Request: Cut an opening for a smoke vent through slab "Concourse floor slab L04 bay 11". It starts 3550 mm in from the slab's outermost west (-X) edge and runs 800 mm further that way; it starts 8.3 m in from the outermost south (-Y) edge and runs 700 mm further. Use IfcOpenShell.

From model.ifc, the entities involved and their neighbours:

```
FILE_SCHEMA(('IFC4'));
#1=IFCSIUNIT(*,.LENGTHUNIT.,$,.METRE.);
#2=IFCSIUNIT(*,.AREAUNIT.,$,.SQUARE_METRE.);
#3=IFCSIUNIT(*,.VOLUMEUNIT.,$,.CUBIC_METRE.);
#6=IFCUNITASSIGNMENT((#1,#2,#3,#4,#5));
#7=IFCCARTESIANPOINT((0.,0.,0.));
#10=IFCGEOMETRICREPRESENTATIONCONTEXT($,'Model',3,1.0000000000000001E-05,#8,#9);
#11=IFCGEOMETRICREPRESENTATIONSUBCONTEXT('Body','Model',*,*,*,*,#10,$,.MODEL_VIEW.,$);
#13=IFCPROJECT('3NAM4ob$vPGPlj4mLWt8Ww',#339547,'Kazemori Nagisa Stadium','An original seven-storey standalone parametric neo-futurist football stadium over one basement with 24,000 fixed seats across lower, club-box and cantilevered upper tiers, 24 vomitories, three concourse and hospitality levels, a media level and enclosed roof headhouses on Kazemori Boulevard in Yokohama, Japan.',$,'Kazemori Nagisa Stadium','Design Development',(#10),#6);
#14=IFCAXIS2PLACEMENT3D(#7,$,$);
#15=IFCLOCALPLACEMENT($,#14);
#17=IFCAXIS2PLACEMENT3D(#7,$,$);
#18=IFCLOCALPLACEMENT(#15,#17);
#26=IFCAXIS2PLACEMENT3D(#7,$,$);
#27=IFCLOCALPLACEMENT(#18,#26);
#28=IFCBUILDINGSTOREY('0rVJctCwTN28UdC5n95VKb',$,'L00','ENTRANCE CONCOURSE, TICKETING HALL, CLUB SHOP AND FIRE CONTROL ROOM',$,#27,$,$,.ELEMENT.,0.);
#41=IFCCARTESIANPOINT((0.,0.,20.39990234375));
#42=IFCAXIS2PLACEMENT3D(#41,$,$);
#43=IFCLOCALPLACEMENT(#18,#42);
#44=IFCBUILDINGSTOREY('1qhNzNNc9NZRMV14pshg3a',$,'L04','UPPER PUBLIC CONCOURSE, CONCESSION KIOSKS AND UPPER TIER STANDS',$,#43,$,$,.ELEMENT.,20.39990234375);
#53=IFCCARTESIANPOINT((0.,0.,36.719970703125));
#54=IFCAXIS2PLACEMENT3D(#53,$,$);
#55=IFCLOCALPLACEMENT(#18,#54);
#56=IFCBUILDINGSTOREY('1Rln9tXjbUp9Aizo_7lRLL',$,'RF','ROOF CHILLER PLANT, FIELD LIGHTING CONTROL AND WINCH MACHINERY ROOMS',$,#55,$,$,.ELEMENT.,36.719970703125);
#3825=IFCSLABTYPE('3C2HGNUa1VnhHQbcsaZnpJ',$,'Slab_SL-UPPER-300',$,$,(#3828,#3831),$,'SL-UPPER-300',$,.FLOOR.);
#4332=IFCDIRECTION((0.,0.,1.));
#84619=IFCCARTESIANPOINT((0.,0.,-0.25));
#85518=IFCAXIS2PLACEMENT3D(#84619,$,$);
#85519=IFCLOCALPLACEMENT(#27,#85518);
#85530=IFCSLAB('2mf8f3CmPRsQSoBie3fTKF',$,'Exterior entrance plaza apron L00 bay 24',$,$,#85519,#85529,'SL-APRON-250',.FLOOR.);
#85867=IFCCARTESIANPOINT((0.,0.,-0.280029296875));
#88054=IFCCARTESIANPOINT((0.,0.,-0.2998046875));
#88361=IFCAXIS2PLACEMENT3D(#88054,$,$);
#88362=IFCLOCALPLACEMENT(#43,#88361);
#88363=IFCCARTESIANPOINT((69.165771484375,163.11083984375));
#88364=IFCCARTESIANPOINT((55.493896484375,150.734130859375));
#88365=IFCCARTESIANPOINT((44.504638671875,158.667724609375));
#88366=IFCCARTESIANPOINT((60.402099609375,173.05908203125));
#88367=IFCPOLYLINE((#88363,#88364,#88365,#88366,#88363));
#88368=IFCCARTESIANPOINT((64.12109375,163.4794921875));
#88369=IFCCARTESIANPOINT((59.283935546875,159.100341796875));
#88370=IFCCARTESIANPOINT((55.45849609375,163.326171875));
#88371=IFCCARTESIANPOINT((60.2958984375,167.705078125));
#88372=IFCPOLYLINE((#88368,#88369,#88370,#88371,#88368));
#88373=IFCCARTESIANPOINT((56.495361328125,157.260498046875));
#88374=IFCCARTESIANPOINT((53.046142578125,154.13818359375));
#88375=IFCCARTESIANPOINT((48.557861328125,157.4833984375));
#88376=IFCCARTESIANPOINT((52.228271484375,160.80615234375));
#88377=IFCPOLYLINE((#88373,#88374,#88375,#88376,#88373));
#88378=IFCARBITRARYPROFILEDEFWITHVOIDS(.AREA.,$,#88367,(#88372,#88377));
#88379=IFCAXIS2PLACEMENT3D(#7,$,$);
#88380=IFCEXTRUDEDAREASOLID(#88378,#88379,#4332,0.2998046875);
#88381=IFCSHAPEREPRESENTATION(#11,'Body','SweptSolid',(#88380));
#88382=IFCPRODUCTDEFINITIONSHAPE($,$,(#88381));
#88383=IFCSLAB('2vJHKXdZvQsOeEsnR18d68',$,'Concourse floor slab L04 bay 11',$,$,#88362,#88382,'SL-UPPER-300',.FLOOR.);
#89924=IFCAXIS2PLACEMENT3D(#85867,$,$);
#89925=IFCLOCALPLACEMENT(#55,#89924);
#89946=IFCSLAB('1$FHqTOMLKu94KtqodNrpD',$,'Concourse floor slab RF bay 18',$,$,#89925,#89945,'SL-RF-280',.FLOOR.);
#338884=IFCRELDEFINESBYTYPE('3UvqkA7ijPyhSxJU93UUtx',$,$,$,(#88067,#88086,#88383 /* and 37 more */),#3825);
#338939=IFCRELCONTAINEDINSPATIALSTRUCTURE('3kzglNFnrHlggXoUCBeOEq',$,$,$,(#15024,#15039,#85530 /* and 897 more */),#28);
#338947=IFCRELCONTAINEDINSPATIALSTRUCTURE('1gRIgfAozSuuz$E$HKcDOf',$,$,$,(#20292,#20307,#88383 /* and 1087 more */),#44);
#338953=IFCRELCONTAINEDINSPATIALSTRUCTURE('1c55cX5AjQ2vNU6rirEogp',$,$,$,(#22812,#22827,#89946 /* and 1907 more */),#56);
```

```python
import numpy as np
import ifcopenshell
import ifcopenshell.api.feature
import ifcopenshell.api.geometry
import ifcopenshell.api.root
import ifcopenshell.geom
import ifcopenshell.util.placement
import ifcopenshell.util.representation
import ifcopenshell.util.shape
import ifcopenshell.util.unit

model = ifcopenshell.open("model.ifc")
unit_scale = ifcopenshell.util.unit.calculate_unit_scale(model)
settings = ifcopenshell.geom.settings()


def volume(element):
    """Net volume in cubic metres, openings subtracted."""
    shape = ifcopenshell.geom.create_shape(settings, element)
    return ifcopenshell.util.shape.get_volume(shape.geometry)


slab = model.by_id(88383)
before = volume(slab)

# Extent in the slab's own axes, in metres. The edges named are its -X and -Y sides.
slab_shape = ifcopenshell.geom.create_shape(settings, slab)
vertices = ifcopenshell.util.shape.get_vertices(slab_shape.geometry)
x_min, y_min, bottom = vertices.min(axis=0)
top = vertices[:, 2].max()

opening = ifcopenshell.api.root.create_entity(model, ifc_class="IfcOpeningElement", name="Smoke vent opening", predefined_type="OPENING")
context = ifcopenshell.util.representation.get_context(model, "Model", "Body", "MODEL_VIEW")
width, depth = 0.8, 0.7
outline = [(0.0, 0.0), (width, 0.0), (width, depth), (0.0, depth), (0.0, 0.0)]
# Overshoot both faces by 50 mm so the cut is clean.
shape = ifcopenshell.api.geometry.add_slab_representation(
    model, context=context, depth=top - bottom + 0.1, polyline=outline
)
ifcopenshell.api.geometry.assign_representation(model, product=opening, representation=shape)

matrix = ifcopenshell.util.placement.get_local_placement(slab.ObjectPlacement)
matrix[:, 3] = matrix @ np.append(np.array([x_min + 3.55, y_min + 8.3, bottom - 0.05]) / unit_scale, 1.0)
ifcopenshell.api.geometry.edit_object_placement(model, product=opening, matrix=matrix, is_si=False)
ifcopenshell.api.feature.add_feature(model, feature=opening, element=slab)

after = volume(slab)

print(f"slab volume {before:.3f} -> {after:.3f} m3")

model.write("model_v2.ifc")
```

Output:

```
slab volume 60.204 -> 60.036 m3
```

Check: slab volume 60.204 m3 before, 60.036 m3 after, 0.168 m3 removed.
